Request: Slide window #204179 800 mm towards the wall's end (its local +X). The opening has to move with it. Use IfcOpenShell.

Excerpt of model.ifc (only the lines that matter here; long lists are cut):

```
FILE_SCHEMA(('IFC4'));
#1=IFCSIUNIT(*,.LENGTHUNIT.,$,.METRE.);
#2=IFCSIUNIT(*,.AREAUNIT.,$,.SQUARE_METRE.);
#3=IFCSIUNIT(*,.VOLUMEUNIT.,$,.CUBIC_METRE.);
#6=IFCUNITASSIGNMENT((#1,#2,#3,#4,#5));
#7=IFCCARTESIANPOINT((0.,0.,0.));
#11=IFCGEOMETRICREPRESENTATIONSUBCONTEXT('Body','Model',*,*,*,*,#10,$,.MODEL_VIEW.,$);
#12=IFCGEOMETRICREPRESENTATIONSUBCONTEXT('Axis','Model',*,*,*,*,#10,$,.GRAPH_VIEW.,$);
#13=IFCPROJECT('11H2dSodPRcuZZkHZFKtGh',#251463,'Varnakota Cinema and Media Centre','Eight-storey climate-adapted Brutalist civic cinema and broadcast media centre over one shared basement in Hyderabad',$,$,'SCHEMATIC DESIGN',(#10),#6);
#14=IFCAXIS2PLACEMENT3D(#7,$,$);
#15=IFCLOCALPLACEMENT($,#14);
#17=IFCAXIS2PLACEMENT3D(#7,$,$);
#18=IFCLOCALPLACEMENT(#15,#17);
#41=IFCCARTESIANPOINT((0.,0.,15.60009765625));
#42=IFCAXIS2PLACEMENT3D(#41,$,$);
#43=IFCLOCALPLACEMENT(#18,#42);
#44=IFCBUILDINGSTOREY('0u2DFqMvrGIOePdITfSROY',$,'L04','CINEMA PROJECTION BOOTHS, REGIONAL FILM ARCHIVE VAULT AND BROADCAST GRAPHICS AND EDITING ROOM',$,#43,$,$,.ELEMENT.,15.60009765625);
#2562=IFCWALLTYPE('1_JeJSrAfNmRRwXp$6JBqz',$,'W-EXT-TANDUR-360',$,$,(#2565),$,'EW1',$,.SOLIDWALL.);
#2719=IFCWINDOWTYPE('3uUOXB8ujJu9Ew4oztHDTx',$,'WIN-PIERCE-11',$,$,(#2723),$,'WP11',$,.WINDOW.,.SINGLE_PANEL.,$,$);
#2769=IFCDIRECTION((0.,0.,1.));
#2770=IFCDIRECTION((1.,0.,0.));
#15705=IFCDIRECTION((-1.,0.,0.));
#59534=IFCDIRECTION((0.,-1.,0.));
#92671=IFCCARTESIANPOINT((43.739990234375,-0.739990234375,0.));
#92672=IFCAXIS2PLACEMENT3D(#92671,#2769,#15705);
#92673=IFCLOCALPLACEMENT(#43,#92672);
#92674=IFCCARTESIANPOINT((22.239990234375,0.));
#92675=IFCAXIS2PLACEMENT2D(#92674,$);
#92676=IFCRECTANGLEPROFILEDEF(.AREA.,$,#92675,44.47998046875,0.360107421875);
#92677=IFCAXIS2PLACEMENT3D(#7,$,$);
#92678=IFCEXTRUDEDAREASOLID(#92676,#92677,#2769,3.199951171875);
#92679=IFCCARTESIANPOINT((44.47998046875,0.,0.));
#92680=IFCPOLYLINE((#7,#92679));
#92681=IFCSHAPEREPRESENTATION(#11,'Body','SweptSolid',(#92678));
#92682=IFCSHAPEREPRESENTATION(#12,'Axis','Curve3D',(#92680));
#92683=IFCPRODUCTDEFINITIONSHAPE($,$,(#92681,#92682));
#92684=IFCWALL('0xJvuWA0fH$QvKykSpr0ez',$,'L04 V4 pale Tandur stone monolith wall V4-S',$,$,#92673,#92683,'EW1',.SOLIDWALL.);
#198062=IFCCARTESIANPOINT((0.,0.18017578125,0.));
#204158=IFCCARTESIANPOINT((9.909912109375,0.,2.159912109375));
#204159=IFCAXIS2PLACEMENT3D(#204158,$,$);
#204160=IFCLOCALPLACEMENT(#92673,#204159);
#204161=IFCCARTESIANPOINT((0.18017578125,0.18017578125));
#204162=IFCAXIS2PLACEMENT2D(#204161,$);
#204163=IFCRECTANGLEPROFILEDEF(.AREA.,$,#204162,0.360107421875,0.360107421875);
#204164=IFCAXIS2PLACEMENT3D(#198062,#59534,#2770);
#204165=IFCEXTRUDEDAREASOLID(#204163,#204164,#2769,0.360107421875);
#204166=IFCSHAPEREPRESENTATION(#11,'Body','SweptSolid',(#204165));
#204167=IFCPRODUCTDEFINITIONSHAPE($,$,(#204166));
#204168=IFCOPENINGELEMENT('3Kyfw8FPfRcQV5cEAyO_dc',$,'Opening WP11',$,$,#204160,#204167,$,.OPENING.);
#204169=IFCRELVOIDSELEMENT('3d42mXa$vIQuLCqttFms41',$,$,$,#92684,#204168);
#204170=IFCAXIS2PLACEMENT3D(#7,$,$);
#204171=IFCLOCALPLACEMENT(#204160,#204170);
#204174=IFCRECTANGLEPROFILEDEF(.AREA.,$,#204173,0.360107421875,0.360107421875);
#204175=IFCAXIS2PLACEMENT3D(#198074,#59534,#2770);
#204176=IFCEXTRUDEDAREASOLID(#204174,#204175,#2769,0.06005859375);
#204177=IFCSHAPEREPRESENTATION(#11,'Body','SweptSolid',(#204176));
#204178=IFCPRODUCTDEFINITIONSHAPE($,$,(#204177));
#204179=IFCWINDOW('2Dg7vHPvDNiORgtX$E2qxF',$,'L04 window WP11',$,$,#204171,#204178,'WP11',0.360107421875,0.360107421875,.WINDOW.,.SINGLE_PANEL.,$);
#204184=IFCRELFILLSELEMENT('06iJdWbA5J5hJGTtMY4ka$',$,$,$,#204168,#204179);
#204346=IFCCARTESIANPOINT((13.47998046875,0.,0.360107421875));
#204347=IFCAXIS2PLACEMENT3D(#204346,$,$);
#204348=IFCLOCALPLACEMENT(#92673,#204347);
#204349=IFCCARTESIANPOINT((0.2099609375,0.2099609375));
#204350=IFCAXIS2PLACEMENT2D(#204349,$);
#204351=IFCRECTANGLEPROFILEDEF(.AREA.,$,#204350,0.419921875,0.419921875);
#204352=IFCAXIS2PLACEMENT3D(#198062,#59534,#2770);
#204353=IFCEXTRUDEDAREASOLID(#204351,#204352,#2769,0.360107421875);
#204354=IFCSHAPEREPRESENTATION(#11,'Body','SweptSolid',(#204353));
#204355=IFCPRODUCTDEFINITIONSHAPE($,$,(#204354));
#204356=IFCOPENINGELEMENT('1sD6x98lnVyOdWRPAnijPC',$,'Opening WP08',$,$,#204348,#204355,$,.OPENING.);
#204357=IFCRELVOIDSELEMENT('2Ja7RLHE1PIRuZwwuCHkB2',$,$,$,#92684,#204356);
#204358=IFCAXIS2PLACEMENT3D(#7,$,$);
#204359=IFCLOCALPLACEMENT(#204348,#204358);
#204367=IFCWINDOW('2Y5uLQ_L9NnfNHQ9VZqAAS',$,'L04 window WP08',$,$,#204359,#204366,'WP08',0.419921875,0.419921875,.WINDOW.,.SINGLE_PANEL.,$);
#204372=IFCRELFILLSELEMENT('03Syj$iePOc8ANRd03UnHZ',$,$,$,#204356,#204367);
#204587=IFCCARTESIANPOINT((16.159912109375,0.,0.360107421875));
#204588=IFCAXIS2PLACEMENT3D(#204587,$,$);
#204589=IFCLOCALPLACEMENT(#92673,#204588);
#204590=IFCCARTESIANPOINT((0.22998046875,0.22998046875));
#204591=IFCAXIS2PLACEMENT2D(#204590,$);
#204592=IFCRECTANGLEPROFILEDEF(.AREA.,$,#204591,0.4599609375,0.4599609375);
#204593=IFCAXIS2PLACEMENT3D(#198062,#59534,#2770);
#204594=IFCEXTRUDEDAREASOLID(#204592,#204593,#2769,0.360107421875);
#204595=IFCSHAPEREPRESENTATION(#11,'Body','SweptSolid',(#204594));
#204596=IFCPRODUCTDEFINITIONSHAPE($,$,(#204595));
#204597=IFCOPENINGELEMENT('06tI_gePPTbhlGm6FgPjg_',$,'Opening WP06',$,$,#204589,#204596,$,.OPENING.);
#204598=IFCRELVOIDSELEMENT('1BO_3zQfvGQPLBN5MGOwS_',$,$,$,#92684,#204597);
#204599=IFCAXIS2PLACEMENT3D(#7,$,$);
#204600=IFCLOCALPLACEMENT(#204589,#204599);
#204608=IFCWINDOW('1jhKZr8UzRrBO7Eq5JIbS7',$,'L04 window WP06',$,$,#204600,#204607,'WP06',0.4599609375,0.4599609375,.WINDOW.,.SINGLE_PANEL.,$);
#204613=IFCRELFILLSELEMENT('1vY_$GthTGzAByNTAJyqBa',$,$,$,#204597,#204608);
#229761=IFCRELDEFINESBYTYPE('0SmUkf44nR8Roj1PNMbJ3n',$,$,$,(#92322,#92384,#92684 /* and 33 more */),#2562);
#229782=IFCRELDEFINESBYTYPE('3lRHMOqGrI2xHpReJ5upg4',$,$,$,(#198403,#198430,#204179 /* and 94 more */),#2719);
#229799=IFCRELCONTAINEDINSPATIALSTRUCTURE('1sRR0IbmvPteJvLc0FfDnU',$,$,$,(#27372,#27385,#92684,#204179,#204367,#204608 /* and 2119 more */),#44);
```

```python
import ifcopenshell
import ifcopenshell.api.geometry
import ifcopenshell.util.placement
import ifcopenshell.util.unit

model = ifcopenshell.open("model.ifc")
unit_scale = ifcopenshell.util.unit.calculate_unit_scale(model)

window = model.by_id(204179)
opening = window.FillsVoids[0].RelatingOpeningElement
wall = opening.VoidsElements[0].RelatingBuildingElement

wall_matrix = ifcopenshell.util.placement.get_local_placement(wall.ObjectPlacement)
shift = wall_matrix[:3, 0] * 0.8 / unit_scale
before = ifcopenshell.util.placement.get_local_placement(window.ObjectPlacement)[:3, 3].copy()

# The window is placed relative to its opening, so it follows when the opening moves.
matrix = ifcopenshell.util.placement.get_local_placement(opening.ObjectPlacement)
matrix[:3, 3] += shift
ifcopenshell.api.geometry.edit_object_placement(
    model, product=opening, matrix=matrix, is_si=False, should_transform_children=True
)

after = ifcopenshell.util.placement.get_local_placement(window.ObjectPlacement)[:3, 3]
print("window moved by", (after - before).round(3) + 0.0)

model.write("model-out.ifc")
```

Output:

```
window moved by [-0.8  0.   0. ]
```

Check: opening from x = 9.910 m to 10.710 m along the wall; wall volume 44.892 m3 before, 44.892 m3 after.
